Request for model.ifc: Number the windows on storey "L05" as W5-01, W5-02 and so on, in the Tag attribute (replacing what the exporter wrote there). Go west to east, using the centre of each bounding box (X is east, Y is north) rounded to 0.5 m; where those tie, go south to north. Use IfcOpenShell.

First a look at what the model holds.

```python
import ifcopenshell
import ifcopenshell.util.element
import ifcopenshell.util.placement

model = ifcopenshell.open("model.ifc")
print(model.schema)
storey = next(s for s in model.by_type("IfcBuildingStorey") if s.Name == "L05")
windows = [e for e in ifcopenshell.util.element.get_decomposition(storey) if e.is_a("IfcWindow")]
for e in sorted(windows, key=lambda e: e.id()):
    origin = ifcopenshell.util.placement.get_local_placement(e.ObjectPlacement)[:3, 3]
    print(e.id(), e.Tag, e.Name, origin.round(2) + 0.0, sep=" | ")
```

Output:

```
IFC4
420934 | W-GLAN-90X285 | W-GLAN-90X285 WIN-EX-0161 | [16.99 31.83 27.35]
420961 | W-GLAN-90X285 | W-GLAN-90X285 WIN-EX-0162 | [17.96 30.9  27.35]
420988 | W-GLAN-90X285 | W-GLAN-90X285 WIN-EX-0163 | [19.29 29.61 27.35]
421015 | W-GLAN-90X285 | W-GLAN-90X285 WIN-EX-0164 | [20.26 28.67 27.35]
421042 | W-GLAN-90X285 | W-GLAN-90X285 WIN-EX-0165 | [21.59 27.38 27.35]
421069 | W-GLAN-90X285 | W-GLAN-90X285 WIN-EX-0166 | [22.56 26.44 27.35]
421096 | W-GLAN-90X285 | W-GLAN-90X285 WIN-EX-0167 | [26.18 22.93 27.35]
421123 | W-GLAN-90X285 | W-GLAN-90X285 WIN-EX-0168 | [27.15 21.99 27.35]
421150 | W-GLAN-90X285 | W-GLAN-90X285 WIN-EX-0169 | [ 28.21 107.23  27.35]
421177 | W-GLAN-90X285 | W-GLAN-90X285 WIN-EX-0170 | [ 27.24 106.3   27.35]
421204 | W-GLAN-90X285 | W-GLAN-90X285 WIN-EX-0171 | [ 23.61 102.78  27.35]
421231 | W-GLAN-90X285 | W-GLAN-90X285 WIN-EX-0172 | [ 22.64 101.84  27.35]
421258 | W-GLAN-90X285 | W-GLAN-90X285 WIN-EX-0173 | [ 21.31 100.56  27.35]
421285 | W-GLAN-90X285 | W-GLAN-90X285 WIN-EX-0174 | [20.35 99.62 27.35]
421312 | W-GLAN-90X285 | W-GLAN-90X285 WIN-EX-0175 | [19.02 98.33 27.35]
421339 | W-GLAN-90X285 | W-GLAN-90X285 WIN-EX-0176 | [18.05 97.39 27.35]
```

```python
import ifcopenshell
import ifcopenshell.geom
import ifcopenshell.util.element
import ifcopenshell.util.shape

model = ifcopenshell.open("model.ifc")
settings = ifcopenshell.geom.settings()
settings.set("use-world-coords", True)


def centre(element):
    shape = ifcopenshell.geom.create_shape(settings, element)
    return ifcopenshell.util.shape.get_bbox_centroid(shape.geometry)


storey = next(s for s in model.by_type("IfcBuildingStorey") if s.Name == "L05")
windows = [e for e in ifcopenshell.util.element.get_decomposition(storey) if e.is_a("IfcWindow")]

# Insertion points can sit at a corner or the storey origin, so sort by the geometry (in metres).
centres = {e: centre(e) for e in windows}
windows.sort(key=lambda e: (round(centres[e][0] / 0.5), centres[e][1]))

for i, e in enumerate(windows, start=1):
    number = f"W5-{i:02d}"
    e.Tag = number
    print(e.id(), number)

model.write("model_updated.ifc")
```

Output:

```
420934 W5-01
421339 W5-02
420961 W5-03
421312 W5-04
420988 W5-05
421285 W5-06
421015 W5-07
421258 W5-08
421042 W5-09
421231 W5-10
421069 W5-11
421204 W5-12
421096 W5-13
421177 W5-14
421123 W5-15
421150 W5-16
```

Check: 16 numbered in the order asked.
